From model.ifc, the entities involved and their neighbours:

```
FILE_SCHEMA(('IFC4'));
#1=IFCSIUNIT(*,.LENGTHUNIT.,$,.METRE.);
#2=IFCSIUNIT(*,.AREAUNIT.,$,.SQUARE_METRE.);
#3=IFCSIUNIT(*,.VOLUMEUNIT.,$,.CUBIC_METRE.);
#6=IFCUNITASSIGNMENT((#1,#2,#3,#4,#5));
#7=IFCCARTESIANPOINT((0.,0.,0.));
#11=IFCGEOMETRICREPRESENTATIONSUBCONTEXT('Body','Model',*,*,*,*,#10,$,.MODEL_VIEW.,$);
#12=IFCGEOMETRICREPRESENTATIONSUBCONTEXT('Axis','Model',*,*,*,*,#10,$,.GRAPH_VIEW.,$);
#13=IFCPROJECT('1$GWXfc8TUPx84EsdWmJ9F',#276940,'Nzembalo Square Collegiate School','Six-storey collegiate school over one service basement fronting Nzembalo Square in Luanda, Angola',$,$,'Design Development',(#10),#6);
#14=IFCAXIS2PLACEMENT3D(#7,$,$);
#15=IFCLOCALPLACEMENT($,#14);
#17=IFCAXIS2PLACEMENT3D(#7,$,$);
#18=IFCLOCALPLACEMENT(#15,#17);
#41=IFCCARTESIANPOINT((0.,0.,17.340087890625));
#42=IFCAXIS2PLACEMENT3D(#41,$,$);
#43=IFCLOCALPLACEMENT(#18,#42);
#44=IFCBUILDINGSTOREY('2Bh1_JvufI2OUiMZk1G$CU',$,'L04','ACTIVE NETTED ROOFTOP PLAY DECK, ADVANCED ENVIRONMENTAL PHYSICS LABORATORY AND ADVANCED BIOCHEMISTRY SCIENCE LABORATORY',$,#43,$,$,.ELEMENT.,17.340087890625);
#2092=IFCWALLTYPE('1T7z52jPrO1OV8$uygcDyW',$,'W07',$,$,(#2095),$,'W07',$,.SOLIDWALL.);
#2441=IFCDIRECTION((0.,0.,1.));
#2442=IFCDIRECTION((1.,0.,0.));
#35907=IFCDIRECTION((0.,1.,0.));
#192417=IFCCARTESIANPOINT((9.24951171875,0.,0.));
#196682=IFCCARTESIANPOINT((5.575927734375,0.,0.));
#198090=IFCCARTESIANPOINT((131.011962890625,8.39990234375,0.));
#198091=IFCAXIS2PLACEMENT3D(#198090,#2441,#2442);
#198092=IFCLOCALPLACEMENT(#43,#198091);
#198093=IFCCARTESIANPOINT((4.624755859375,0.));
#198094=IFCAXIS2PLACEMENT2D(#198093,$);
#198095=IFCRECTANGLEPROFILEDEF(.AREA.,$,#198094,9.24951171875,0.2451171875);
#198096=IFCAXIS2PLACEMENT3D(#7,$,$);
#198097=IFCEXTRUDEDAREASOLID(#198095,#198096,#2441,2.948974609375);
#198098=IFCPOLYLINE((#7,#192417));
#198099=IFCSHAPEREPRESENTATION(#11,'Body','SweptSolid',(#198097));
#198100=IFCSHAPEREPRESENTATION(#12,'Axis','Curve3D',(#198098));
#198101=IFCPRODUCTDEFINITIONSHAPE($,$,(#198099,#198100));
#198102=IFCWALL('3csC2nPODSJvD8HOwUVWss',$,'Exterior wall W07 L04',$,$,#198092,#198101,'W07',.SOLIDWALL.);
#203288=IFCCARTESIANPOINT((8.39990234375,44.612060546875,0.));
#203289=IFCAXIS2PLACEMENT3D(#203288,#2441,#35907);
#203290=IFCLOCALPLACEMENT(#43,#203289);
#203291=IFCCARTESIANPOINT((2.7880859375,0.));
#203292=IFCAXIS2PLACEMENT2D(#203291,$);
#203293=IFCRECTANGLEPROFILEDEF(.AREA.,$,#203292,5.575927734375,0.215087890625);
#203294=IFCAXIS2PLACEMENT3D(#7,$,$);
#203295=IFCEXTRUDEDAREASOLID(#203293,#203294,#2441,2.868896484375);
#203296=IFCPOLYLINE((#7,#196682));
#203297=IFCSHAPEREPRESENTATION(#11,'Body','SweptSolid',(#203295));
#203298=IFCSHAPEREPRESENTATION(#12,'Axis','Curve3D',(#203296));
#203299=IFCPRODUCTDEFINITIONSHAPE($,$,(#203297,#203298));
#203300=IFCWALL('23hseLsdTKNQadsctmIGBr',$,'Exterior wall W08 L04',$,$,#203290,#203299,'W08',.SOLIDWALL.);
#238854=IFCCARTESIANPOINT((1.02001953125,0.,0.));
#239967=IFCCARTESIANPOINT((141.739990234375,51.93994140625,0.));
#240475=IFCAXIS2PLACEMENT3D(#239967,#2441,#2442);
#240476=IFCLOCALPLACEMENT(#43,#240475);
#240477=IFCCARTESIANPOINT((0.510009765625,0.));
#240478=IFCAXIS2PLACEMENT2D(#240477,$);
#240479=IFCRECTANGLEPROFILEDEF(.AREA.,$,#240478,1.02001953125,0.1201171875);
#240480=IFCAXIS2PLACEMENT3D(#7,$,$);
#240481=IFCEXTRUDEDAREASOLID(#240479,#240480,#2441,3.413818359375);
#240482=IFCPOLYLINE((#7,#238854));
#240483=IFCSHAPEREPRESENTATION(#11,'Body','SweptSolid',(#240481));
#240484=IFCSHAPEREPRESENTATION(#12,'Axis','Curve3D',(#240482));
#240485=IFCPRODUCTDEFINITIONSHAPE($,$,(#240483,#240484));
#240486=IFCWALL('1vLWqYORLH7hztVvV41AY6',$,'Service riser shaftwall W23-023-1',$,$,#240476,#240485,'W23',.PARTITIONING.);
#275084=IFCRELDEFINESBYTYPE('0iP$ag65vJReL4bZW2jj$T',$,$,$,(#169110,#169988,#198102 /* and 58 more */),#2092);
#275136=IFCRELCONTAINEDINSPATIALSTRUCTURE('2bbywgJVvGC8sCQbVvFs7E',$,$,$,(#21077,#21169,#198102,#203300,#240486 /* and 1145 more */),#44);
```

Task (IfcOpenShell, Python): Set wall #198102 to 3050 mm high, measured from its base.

```python
import ifcopenshell
import ifcopenshell.geom
import ifcopenshell.util.representation
import ifcopenshell.util.shape

model = ifcopenshell.open("model.ifc")
settings = ifcopenshell.geom.settings()


def volume(element):
    """Net volume in cubic metres, openings subtracted."""
    shape = ifcopenshell.geom.create_shape(settings, element)
    return ifcopenshell.util.shape.get_volume(shape.geometry)


wall = model.by_guid("3csC2nPODSJvD8HOwUVWss")
before = volume(wall)

body = ifcopenshell.util.representation.get_representation(wall, "Model", "Body")
solid = body.Items[0]
old_height = solid.Depth
solid.Depth = 3.05
after = volume(wall)

print(f"height {old_height:g} -> {solid.Depth:g}, volume {before:.3f} -> {after:.3f} m3")

model.write("model_v2.ifc")
```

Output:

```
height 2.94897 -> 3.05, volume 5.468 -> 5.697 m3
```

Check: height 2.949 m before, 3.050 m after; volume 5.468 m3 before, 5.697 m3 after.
